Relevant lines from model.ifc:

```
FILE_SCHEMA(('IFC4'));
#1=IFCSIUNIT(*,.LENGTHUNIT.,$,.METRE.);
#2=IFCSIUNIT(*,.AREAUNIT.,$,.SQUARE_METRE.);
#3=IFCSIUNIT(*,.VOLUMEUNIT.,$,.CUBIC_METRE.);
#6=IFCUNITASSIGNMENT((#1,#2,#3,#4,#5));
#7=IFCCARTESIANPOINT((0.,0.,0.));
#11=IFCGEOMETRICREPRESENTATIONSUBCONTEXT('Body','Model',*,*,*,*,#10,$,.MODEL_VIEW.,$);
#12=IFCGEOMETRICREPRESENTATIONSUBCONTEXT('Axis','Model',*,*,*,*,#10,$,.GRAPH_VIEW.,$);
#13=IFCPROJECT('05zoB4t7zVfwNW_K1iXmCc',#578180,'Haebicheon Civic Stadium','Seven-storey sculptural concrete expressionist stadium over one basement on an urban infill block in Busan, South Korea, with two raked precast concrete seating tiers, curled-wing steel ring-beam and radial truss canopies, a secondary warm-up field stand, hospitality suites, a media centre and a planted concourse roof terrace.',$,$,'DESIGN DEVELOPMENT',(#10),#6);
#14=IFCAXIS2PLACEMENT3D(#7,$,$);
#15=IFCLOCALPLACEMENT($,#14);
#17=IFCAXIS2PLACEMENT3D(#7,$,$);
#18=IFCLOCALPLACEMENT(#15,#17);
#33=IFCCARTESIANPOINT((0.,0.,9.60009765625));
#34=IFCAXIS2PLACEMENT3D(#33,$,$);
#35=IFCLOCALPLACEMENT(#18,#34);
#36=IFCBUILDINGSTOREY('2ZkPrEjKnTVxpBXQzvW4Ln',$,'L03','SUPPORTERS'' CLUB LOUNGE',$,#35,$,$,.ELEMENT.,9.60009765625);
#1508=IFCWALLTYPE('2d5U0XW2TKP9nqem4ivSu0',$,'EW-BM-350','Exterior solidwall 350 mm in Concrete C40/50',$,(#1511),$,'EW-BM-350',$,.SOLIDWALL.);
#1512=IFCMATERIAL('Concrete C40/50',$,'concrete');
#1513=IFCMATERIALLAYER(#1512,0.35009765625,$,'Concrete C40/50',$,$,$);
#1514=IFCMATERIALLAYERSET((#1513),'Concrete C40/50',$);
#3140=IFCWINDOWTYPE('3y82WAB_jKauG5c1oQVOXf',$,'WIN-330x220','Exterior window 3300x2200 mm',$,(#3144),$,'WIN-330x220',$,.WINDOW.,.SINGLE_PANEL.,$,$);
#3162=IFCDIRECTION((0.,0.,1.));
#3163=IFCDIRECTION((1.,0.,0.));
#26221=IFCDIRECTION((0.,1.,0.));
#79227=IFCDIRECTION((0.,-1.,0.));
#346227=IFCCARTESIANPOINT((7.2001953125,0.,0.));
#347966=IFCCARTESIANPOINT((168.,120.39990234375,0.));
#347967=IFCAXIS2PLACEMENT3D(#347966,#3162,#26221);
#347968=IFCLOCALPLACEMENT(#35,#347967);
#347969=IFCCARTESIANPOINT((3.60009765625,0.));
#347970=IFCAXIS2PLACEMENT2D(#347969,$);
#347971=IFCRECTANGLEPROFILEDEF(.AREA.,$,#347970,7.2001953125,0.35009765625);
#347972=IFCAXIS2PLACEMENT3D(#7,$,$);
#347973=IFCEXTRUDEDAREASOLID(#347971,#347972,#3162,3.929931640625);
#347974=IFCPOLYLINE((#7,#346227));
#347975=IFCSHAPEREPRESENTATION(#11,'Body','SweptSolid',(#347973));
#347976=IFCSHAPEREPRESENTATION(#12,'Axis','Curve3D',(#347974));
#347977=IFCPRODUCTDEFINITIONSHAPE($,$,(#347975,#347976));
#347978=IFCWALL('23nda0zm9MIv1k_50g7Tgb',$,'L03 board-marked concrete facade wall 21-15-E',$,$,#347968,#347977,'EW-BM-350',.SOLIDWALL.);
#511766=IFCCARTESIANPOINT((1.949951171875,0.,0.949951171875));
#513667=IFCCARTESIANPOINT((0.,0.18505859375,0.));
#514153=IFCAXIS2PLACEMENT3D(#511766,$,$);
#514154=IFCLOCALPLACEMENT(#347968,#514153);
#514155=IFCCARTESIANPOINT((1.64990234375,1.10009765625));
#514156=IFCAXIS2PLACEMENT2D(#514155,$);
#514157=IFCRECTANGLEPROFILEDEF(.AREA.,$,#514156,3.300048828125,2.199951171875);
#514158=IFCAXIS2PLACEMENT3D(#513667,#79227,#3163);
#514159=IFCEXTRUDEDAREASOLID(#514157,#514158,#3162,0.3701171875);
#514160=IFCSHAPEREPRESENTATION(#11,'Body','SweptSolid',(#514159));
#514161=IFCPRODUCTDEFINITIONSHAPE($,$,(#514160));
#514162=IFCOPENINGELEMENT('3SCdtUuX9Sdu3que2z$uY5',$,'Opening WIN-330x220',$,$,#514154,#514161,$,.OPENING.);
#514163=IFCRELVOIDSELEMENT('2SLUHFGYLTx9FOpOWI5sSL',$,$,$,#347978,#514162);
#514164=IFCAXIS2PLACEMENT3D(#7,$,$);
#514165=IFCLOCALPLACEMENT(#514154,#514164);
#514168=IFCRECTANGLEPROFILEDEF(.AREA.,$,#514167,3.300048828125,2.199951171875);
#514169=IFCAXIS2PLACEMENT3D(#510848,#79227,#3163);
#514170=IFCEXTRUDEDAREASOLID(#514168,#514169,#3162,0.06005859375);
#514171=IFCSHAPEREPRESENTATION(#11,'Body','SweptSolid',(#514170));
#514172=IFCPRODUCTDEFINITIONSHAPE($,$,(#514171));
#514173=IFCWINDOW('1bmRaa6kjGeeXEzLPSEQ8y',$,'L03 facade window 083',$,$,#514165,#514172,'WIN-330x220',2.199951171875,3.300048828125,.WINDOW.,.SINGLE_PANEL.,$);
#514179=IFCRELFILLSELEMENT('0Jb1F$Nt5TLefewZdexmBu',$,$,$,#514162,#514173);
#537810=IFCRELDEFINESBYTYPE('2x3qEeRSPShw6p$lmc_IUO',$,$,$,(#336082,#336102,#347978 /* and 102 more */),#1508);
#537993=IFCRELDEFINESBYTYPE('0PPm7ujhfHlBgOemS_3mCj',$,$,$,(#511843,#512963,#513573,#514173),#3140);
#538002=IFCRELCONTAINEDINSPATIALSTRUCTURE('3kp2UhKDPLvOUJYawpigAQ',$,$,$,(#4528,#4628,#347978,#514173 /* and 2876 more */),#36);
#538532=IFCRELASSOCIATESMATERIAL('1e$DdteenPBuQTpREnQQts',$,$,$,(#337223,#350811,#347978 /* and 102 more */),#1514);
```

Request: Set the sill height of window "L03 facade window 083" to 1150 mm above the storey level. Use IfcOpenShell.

```python
import numpy as np
import ifcopenshell
import ifcopenshell.api.geometry
import ifcopenshell.geom
import ifcopenshell.util.element
import ifcopenshell.util.placement
import ifcopenshell.util.shape
import ifcopenshell.util.unit

model = ifcopenshell.open("model.ifc")
unit_scale = ifcopenshell.util.unit.calculate_unit_scale(model)

window = model.by_guid("1bmRaa6kjGeeXEzLPSEQ8y")
opening = window.FillsVoids[0].RelatingOpeningElement
storey = ifcopenshell.util.element.get_container(window, ifc_class="IfcBuildingStorey")
level = ifcopenshell.util.placement.get_local_placement(storey.ObjectPlacement)[2, 3]

# The opening's origin need not be at the sill, so measure its lowest point.
shape = ifcopenshell.geom.create_shape(ifcopenshell.geom.settings(), opening)
bottom = ifcopenshell.util.shape.get_shape_bottom_elevation(shape, shape.geometry) / unit_scale
dz = level + 1.15 - bottom

shift = np.array([0.0, 0.0, dz])
# The window is placed relative to its opening, so it follows when the opening moves.
matrix = ifcopenshell.util.placement.get_local_placement(opening.ObjectPlacement)
matrix[:3, 3] += shift
ifcopenshell.api.geometry.edit_object_placement(
    model, product=opening, matrix=matrix, is_si=False, should_transform_children=True
)

print(f"moved by {dz * unit_scale:+.3f} m")

model.write("model_edited.ifc")
```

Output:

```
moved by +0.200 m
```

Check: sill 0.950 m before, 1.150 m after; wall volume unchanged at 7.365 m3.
